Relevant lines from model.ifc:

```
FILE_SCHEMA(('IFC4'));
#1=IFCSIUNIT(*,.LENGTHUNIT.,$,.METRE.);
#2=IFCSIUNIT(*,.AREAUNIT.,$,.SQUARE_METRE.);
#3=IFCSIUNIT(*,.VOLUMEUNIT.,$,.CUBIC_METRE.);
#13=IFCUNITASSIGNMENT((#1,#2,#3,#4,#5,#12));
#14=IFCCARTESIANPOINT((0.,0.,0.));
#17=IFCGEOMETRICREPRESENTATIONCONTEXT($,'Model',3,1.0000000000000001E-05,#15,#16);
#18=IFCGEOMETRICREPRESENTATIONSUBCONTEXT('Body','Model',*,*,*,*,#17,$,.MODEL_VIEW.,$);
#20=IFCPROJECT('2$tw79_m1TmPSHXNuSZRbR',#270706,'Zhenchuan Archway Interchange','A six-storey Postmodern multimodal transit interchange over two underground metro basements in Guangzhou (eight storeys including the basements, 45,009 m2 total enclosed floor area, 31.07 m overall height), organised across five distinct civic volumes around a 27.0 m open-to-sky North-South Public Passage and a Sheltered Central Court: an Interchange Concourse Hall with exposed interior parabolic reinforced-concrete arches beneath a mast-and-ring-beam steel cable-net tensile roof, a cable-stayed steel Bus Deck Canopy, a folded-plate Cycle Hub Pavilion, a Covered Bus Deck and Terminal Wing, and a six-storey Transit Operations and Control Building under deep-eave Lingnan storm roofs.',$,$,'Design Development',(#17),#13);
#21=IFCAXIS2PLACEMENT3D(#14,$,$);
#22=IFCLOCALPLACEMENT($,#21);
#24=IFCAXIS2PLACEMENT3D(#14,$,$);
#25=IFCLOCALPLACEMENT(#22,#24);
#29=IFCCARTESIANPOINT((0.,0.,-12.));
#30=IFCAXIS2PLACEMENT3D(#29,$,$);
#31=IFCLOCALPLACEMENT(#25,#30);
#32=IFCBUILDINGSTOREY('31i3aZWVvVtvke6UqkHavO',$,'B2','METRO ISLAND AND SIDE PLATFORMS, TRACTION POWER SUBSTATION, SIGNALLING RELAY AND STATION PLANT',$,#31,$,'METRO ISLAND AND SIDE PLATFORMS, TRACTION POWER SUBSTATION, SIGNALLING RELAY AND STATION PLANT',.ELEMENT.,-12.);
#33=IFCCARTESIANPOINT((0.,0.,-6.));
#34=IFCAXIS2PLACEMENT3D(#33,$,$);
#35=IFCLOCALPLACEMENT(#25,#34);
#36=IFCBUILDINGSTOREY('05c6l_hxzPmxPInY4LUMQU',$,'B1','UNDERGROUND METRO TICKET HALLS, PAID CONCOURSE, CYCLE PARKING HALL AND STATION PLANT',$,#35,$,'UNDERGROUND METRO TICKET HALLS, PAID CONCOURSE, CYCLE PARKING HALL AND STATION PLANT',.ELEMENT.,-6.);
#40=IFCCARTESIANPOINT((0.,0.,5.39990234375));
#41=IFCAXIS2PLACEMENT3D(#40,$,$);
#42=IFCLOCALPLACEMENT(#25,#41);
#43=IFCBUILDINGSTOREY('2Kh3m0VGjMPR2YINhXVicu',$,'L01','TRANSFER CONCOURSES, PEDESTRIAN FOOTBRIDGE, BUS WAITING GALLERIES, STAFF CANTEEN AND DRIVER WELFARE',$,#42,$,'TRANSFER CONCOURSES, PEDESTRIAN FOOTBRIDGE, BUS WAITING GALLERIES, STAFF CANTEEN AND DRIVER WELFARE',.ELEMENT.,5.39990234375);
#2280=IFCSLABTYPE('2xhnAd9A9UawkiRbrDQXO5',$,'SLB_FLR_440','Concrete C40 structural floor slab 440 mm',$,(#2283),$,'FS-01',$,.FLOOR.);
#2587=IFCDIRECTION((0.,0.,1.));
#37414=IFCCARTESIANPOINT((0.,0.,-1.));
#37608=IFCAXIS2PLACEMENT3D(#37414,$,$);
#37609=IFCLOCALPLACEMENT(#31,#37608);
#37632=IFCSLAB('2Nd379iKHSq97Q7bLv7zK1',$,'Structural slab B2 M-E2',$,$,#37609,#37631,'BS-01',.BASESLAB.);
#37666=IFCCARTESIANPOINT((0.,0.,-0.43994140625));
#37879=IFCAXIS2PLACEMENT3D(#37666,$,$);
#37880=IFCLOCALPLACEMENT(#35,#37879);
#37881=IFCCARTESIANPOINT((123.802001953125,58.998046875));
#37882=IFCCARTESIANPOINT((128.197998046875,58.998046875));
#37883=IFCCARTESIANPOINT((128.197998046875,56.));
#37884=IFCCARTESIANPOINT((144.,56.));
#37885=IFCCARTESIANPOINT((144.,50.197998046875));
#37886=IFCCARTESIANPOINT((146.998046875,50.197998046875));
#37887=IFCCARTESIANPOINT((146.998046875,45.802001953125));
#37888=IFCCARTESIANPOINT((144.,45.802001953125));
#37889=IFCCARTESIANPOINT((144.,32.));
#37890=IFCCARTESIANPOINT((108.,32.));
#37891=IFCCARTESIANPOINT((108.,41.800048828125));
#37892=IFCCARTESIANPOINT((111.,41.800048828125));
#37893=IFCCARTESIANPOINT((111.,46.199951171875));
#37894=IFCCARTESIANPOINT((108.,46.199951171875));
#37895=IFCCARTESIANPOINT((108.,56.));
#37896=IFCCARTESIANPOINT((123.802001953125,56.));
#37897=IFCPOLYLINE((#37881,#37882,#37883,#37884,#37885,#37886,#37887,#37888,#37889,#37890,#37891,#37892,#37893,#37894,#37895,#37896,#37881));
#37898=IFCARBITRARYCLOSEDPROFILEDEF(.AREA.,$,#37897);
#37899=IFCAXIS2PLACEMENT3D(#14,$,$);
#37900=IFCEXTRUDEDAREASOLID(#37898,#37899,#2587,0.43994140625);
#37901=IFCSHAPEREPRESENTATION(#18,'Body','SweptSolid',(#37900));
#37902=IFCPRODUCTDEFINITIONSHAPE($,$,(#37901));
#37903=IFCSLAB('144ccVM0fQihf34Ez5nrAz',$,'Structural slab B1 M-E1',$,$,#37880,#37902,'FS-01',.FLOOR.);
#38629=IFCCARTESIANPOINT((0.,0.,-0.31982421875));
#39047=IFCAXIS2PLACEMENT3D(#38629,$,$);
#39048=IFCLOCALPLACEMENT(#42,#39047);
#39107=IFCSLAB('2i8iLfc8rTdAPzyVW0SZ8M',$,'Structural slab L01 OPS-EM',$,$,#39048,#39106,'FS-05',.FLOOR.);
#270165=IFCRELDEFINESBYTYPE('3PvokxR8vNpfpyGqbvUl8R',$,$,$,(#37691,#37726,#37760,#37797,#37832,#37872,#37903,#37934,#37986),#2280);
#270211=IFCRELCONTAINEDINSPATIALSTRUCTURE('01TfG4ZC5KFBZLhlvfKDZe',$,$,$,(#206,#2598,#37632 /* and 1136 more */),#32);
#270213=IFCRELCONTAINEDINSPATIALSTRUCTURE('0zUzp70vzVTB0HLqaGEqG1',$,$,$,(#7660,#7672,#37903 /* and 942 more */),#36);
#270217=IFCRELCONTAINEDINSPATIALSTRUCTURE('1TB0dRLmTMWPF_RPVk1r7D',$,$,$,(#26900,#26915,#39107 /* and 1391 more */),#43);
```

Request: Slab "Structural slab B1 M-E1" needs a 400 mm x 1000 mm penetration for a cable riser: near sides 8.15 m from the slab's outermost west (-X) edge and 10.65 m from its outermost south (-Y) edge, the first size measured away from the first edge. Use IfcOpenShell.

```python
import numpy as np
import ifcopenshell
import ifcopenshell.api.feature
import ifcopenshell.api.geometry
import ifcopenshell.api.root
import ifcopenshell.geom
import ifcopenshell.util.placement
import ifcopenshell.util.representation
import ifcopenshell.util.shape
import ifcopenshell.util.unit

model = ifcopenshell.open("model.ifc")
unit_scale = ifcopenshell.util.unit.calculate_unit_scale(model)
settings = ifcopenshell.geom.settings()


def volume(element):
    """Net volume in cubic metres, openings subtracted."""
    shape = ifcopenshell.geom.create_shape(settings, element)
    return ifcopenshell.util.shape.get_volume(shape.geometry)


slab = model.by_guid("144ccVM0fQihf34Ez5nrAz")
before = volume(slab)

# Extent in the slab's own axes, in metres. The edges named are its -X and -Y sides.
slab_shape = ifcopenshell.geom.create_shape(settings, slab)
vertices = ifcopenshell.util.shape.get_vertices(slab_shape.geometry)
x_min, y_min, bottom = vertices.min(axis=0)
top = vertices[:, 2].max()

opening = ifcopenshell.api.root.create_entity(model, ifc_class="IfcOpeningElement", name="Cable riser opening", predefined_type="OPENING")
context = ifcopenshell.util.representation.get_context(model, "Model", "Body", "MODEL_VIEW")
width, depth = 0.4, 1
outline = [(0.0, 0.0), (width, 0.0), (width, depth), (0.0, depth), (0.0, 0.0)]
# Overshoot both faces by 50 mm so the cut is clean.
shape = ifcopenshell.api.geometry.add_slab_representation(
    model, context=context, depth=top - bottom + 0.1, polyline=outline
)
ifcopenshell.api.geometry.assign_representation(model, product=opening, representation=shape)

matrix = ifcopenshell.util.placement.get_local_placement(slab.ObjectPlacement)
matrix[:, 3] = matrix @ np.append(np.array([x_min + 8.15, y_min + 10.65, bottom - 0.05]) / unit_scale, 1.0)
ifcopenshell.api.geometry.edit_object_placement(model, product=opening, matrix=matrix, is_si=False)
ifcopenshell.api.feature.add_feature(model, feature=opening, element=slab)

after = volume(slab)

print(f"slab volume {before:.3f} -> {after:.3f} m3")

model.write("model_updated.ifc")
```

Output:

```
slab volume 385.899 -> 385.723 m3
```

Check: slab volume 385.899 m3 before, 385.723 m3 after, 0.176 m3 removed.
